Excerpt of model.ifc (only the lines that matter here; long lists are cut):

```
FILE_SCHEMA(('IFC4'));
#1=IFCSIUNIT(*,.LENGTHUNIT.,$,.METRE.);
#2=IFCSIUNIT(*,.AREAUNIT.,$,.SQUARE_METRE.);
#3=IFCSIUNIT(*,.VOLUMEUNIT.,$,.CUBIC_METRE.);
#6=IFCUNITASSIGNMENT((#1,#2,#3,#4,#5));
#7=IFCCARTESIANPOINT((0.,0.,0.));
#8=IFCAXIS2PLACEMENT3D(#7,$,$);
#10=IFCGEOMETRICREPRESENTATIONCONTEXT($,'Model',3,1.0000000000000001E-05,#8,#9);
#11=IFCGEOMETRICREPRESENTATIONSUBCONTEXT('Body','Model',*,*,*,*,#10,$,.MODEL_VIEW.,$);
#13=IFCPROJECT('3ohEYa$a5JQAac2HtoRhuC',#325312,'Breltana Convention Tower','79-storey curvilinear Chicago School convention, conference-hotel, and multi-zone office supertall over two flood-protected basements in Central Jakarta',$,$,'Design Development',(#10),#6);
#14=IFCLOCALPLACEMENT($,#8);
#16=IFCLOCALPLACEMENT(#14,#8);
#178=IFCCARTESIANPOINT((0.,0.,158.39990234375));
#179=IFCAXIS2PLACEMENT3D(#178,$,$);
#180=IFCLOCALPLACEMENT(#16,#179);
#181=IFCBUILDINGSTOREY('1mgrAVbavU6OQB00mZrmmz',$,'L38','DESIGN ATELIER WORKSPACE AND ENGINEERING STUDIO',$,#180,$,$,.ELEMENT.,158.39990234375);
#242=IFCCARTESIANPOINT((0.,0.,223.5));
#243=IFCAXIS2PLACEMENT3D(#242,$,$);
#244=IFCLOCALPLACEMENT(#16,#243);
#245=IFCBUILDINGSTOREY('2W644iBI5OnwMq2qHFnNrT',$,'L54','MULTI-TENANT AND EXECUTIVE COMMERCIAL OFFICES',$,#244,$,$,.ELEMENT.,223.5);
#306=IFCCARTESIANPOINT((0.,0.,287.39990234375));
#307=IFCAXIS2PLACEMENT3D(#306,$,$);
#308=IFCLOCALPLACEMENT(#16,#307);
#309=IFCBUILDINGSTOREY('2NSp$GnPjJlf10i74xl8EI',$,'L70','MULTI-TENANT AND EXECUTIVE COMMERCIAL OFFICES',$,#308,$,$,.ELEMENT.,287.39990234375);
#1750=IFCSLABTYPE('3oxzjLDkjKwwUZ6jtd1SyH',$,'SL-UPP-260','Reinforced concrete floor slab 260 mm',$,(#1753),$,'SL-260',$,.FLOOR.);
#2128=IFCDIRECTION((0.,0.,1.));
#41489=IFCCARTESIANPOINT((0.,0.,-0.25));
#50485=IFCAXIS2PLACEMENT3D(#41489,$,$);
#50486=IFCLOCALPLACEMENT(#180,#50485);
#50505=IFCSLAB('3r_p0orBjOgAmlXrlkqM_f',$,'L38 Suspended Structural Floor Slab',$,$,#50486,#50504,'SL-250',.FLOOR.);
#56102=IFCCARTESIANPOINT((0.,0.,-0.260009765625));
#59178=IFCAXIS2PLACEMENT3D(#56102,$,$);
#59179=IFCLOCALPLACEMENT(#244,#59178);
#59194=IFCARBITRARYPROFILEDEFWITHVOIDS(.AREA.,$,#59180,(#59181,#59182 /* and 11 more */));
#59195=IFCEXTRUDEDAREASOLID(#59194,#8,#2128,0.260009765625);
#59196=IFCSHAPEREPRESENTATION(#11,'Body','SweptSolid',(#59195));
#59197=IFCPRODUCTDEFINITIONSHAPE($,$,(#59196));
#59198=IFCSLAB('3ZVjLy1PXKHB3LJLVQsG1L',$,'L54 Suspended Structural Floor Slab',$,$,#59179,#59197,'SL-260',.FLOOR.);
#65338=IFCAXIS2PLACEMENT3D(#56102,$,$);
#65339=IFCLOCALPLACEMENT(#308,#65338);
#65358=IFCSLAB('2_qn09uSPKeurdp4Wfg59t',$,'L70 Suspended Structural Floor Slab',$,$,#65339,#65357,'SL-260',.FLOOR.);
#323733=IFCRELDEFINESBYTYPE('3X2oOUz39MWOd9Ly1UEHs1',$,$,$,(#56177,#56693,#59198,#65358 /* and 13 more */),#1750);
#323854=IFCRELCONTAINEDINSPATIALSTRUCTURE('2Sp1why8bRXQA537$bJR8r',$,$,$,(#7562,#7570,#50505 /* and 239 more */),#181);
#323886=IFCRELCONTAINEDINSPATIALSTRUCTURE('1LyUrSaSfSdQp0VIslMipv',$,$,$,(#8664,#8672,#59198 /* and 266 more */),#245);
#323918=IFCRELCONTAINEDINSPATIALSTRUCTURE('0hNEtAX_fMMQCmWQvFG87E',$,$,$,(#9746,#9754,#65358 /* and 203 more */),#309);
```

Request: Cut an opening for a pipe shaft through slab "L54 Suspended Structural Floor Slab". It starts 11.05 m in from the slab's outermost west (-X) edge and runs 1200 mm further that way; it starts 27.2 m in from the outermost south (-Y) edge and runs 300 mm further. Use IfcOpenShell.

```python
import numpy as np
import ifcopenshell
import ifcopenshell.api.feature
import ifcopenshell.api.geometry
import ifcopenshell.api.root
import ifcopenshell.geom
import ifcopenshell.util.placement
import ifcopenshell.util.representation
import ifcopenshell.util.shape
import ifcopenshell.util.unit

model = ifcopenshell.open("model.ifc")
unit_scale = ifcopenshell.util.unit.calculate_unit_scale(model)
settings = ifcopenshell.geom.settings()


def volume(element):
    """Net volume in cubic metres, openings subtracted."""
    shape = ifcopenshell.geom.create_shape(settings, element)
    return ifcopenshell.util.shape.get_volume(shape.geometry)


slab = model.by_guid("3ZVjLy1PXKHB3LJLVQsG1L")
before = volume(slab)

# Extent in the slab's own axes, in metres. The edges named are its -X and -Y sides.
slab_shape = ifcopenshell.geom.create_shape(settings, slab)
vertices = ifcopenshell.util.shape.get_vertices(slab_shape.geometry)
x_min, y_min, bottom = vertices.min(axis=0)
top = vertices[:, 2].max()

opening = ifcopenshell.api.root.create_entity(model, ifc_class="IfcOpeningElement", name="Pipe shaft opening", predefined_type="OPENING")
context = ifcopenshell.util.representation.get_context(model, "Model", "Body", "MODEL_VIEW")
width, depth = 1.2, 0.3
outline = [(0.0, 0.0), (width, 0.0), (width, depth), (0.0, depth), (0.0, 0.0)]
# Overshoot both faces by 50 mm so the cut is clean.
shape = ifcopenshell.api.geometry.add_slab_representation(
    model, context=context, depth=top - bottom + 0.1, polyline=outline
)
ifcopenshell.api.geometry.assign_representation(model, product=opening, representation=shape)

matrix = ifcopenshell.util.placement.get_local_placement(slab.ObjectPlacement)
matrix[:, 3] = matrix @ np.append(np.array([x_min + 11.05, y_min + 27.2, bottom - 0.05]) / unit_scale, 1.0)
ifcopenshell.api.geometry.edit_object_placement(model, product=opening, matrix=matrix, is_si=False)
ifcopenshell.api.feature.add_feature(model, feature=opening, element=slab)

after = volume(slab)

print(f"slab volume {before:.3f} -> {after:.3f} m3")

model.write("model_edited.ifc")
```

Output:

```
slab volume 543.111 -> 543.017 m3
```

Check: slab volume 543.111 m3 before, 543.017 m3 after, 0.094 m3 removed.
